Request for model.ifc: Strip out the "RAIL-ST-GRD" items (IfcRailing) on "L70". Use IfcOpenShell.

First a look at what the model holds.

```python
import ifcopenshell
import ifcopenshell.util.element

model = ifcopenshell.open("model.ifc")
print(model.schema)
storey = next(s for s in model.by_type("IfcBuildingStorey") if s.Name == "L70")
railings = [e for e in ifcopenshell.util.element.get_decomposition(storey) if e.is_a("IfcRailing")]
seen = {}
for e in railings:
    element_type = ifcopenshell.util.element.get_type(e)
    name = element_type.Name if element_type not in (None, e) else None
    seen[name] = seen.get(name, 0) + 1
for name, count in sorted(seen.items(), key=str):
    print(count, "x", name)
```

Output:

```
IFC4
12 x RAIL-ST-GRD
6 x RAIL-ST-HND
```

```python
import ifcopenshell
import ifcopenshell.api.root
import ifcopenshell.util.element

model = ifcopenshell.open("model.ifc")

storey = next(s for s in model.by_type("IfcBuildingStorey") if s.Name == "L70")
railings = [e for e in ifcopenshell.util.element.get_decomposition(storey) if e.is_a("IfcRailing")]
targets = [e for e in railings if (t := ifcopenshell.util.element.get_type(e)) not in (None, e) and t.Name == "RAIL-ST-GRD"]

for e in targets:
    ifcopenshell.api.root.remove_product(model, product=e)
print(len(targets), "removed")

model.write("model-out.ifc")
```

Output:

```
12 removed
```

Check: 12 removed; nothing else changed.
